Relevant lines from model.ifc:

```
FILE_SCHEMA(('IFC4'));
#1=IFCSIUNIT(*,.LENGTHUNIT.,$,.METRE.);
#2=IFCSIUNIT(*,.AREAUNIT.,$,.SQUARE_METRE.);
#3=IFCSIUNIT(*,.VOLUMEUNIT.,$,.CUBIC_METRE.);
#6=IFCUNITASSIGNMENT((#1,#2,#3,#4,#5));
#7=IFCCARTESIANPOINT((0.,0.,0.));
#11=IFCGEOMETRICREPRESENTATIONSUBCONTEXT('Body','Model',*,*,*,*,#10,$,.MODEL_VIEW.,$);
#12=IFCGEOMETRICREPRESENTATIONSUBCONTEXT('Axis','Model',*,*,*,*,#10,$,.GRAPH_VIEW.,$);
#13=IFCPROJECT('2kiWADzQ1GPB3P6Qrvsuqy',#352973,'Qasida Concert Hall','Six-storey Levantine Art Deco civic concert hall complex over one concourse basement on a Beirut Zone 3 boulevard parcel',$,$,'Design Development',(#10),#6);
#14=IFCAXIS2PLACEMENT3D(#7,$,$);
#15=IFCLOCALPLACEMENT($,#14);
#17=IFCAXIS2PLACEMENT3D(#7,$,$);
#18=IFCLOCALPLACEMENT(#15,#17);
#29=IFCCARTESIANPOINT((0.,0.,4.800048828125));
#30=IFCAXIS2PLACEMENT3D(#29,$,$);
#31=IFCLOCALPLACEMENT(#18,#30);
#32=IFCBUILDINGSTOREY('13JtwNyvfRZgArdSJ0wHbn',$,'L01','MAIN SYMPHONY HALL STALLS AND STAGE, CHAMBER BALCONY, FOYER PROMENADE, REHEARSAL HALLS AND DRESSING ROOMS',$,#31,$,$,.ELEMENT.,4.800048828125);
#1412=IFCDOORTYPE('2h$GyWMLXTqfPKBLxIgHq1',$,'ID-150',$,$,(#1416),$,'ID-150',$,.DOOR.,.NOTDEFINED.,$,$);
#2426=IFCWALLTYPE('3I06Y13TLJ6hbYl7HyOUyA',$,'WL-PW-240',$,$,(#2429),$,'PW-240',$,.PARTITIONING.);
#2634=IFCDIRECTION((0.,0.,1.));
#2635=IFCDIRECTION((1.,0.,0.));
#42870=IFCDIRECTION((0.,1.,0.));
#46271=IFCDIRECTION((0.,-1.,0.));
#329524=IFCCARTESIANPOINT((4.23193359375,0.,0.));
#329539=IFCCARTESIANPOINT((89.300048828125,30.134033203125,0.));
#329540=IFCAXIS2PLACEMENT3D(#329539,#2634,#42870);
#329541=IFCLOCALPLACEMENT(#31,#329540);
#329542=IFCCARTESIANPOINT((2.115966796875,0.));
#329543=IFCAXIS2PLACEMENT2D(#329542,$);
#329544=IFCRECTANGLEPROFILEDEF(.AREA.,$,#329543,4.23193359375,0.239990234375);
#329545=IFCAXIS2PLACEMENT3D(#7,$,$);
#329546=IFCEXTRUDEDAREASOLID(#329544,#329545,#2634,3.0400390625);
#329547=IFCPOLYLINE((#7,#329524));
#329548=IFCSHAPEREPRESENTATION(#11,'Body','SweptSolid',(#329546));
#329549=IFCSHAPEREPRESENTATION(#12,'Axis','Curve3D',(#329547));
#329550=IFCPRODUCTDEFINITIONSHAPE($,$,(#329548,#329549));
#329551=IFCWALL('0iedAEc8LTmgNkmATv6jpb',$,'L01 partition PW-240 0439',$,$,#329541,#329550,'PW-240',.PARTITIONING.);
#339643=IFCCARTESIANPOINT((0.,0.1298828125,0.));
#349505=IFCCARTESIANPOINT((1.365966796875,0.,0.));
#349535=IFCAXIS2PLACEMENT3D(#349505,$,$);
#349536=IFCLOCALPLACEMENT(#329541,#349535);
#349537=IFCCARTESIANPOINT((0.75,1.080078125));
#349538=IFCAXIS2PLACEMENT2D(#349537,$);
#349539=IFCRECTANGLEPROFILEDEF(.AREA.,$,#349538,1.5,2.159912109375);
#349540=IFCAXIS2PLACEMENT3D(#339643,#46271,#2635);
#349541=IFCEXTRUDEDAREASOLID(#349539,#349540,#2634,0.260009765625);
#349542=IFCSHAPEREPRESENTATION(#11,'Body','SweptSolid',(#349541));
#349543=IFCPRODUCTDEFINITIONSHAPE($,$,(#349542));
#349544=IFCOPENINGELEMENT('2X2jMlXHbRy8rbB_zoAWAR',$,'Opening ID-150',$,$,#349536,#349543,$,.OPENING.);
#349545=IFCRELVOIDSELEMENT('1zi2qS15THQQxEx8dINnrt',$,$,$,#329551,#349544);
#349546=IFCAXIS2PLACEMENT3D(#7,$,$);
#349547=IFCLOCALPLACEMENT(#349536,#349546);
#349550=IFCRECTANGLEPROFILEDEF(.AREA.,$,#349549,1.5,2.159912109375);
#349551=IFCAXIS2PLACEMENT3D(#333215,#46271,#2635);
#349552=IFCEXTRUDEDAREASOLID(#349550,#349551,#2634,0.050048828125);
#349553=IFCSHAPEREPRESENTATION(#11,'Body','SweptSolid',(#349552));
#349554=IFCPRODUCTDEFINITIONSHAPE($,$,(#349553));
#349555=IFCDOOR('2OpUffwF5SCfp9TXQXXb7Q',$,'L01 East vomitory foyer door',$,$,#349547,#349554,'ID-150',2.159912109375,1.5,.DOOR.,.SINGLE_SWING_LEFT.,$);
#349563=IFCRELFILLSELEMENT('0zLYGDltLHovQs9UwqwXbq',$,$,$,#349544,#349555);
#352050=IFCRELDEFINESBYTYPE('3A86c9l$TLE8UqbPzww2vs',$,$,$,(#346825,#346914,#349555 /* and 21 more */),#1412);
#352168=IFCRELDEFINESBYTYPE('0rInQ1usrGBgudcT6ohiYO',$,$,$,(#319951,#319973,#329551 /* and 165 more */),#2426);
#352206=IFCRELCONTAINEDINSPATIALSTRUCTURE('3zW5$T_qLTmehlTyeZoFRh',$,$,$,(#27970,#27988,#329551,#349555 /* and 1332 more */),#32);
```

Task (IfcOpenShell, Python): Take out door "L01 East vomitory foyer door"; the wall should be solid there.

```python
import ifcopenshell
import ifcopenshell.api.feature
import ifcopenshell.api.root
import ifcopenshell.geom
import ifcopenshell.util.shape

model = ifcopenshell.open("model.ifc")
settings = ifcopenshell.geom.settings()


def volume(element):
    """Net volume in cubic metres, openings subtracted."""
    shape = ifcopenshell.geom.create_shape(settings, element)
    return ifcopenshell.util.shape.get_volume(shape.geometry)


door = model.by_id(349555)
opening = door.FillsVoids[0].RelatingOpeningElement
wall = opening.VoidsElements[0].RelatingBuildingElement
before = volume(wall)

ifcopenshell.api.root.remove_product(model, product=door)
ifcopenshell.api.feature.remove_feature(model, feature=opening)

after = volume(wall)

print(f"wall volume {before:.3f} -> {after:.3f} m3")

model.write("model_edited.ifc")
```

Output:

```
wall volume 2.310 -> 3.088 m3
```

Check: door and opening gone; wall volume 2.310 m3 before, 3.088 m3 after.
